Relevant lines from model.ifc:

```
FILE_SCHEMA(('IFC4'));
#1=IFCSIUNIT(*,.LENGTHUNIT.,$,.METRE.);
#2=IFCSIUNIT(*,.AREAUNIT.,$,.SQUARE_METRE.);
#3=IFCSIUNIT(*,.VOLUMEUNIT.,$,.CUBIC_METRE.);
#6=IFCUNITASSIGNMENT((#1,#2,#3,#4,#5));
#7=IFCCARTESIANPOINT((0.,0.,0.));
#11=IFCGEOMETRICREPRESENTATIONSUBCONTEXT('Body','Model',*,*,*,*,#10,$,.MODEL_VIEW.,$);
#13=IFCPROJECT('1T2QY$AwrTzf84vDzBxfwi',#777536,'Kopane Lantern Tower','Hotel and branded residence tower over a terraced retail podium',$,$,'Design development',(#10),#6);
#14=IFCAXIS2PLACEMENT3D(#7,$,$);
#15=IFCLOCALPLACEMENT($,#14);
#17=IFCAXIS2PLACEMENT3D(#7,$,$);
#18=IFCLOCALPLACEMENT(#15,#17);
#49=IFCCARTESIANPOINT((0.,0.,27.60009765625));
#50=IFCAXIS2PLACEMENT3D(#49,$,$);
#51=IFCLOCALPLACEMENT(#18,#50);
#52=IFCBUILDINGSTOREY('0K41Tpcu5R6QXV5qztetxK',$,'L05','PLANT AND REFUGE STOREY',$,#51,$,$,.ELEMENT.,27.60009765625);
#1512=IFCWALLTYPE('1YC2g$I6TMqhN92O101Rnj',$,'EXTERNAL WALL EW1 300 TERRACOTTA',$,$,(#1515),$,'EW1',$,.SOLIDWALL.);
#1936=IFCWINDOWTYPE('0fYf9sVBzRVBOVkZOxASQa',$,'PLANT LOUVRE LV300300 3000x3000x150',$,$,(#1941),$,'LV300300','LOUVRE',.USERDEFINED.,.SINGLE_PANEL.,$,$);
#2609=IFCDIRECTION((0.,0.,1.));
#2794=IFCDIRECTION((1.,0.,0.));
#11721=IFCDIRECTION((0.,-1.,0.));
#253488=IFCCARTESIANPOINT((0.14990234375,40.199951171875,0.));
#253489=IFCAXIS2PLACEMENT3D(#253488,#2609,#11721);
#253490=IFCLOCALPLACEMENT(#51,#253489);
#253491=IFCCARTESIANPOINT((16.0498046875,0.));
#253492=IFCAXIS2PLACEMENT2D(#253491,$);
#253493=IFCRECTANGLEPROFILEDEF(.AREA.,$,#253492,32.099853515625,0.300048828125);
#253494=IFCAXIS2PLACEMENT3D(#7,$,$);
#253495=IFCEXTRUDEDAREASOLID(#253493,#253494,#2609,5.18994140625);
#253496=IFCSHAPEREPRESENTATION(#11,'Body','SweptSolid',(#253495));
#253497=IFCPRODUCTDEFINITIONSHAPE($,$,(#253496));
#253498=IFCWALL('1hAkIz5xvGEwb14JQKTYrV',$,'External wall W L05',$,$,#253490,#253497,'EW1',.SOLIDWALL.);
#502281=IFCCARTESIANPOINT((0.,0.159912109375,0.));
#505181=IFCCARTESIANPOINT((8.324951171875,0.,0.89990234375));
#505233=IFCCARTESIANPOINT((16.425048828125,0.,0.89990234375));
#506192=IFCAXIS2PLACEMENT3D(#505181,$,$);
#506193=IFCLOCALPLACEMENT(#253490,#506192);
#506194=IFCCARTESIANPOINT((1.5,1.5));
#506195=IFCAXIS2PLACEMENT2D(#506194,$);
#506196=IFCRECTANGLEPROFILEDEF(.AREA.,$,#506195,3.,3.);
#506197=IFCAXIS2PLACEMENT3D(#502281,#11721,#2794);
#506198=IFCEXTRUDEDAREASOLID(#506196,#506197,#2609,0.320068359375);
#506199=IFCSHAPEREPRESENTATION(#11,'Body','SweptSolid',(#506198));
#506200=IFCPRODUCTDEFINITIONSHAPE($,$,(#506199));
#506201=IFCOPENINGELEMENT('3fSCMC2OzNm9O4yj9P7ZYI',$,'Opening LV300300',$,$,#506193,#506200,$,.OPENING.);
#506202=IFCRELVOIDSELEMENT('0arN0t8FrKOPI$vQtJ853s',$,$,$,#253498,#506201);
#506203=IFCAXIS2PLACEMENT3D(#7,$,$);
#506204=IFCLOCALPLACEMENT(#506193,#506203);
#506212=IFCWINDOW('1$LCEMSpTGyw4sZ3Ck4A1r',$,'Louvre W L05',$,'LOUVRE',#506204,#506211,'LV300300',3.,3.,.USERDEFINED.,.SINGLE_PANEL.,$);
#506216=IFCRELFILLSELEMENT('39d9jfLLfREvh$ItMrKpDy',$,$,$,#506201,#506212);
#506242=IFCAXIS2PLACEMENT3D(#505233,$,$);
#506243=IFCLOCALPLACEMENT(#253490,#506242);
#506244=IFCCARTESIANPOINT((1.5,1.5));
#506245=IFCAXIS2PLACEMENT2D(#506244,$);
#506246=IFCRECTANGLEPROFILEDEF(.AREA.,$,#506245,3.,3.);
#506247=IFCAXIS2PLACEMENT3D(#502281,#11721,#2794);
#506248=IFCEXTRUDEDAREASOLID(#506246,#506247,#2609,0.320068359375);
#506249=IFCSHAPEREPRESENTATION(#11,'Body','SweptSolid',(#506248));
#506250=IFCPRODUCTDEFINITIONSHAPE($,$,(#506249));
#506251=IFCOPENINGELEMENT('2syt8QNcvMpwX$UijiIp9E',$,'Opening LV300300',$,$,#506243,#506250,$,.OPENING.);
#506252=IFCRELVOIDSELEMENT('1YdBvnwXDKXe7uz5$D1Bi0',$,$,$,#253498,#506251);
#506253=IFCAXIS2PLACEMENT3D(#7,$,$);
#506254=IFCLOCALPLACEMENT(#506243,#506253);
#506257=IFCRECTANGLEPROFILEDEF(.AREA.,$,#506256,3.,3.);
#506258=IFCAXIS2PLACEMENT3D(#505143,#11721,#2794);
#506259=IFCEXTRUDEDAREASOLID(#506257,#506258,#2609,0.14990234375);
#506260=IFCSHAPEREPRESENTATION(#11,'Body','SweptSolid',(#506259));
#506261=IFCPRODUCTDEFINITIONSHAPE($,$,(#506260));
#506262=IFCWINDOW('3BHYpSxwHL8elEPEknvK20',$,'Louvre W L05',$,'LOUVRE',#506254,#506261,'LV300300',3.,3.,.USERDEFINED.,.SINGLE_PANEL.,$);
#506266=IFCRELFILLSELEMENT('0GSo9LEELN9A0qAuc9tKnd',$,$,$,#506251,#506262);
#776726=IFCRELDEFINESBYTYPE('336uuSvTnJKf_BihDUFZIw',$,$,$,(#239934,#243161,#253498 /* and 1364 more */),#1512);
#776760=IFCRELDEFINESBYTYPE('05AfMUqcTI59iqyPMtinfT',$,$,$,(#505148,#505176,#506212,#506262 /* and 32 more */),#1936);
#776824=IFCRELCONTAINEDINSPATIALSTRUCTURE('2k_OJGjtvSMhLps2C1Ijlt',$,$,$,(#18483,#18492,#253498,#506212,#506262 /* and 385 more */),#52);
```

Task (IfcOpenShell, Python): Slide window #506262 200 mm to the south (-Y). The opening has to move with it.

```python
import ifcopenshell
import ifcopenshell.api.geometry
import ifcopenshell.util.placement
import ifcopenshell.util.unit

model = ifcopenshell.open("model.ifc")
unit_scale = ifcopenshell.util.unit.calculate_unit_scale(model)

window = model.by_guid("3BHYpSxwHL8elEPEknvK20")
opening = window.FillsVoids[0].RelatingOpeningElement
wall = opening.VoidsElements[0].RelatingBuildingElement

wall_matrix = ifcopenshell.util.placement.get_local_placement(wall.ObjectPlacement)
shift = wall_matrix[:3, 0] * 0.2 / unit_scale
before = ifcopenshell.util.placement.get_local_placement(window.ObjectPlacement)[:3, 3].copy()

# The window is placed relative to its opening, so it follows when the opening moves.
matrix = ifcopenshell.util.placement.get_local_placement(opening.ObjectPlacement)
matrix[:3, 3] += shift
ifcopenshell.api.geometry.edit_object_placement(
    model, product=opening, matrix=matrix, is_si=False, should_transform_children=True
)

after = ifcopenshell.util.placement.get_local_placement(window.ObjectPlacement)[:3, 3]
print("window moved by", (after - before).round(3) + 0.0)

model.write("model-out.ifc")
```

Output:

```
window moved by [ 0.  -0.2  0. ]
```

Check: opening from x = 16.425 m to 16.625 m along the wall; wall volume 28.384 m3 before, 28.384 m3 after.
